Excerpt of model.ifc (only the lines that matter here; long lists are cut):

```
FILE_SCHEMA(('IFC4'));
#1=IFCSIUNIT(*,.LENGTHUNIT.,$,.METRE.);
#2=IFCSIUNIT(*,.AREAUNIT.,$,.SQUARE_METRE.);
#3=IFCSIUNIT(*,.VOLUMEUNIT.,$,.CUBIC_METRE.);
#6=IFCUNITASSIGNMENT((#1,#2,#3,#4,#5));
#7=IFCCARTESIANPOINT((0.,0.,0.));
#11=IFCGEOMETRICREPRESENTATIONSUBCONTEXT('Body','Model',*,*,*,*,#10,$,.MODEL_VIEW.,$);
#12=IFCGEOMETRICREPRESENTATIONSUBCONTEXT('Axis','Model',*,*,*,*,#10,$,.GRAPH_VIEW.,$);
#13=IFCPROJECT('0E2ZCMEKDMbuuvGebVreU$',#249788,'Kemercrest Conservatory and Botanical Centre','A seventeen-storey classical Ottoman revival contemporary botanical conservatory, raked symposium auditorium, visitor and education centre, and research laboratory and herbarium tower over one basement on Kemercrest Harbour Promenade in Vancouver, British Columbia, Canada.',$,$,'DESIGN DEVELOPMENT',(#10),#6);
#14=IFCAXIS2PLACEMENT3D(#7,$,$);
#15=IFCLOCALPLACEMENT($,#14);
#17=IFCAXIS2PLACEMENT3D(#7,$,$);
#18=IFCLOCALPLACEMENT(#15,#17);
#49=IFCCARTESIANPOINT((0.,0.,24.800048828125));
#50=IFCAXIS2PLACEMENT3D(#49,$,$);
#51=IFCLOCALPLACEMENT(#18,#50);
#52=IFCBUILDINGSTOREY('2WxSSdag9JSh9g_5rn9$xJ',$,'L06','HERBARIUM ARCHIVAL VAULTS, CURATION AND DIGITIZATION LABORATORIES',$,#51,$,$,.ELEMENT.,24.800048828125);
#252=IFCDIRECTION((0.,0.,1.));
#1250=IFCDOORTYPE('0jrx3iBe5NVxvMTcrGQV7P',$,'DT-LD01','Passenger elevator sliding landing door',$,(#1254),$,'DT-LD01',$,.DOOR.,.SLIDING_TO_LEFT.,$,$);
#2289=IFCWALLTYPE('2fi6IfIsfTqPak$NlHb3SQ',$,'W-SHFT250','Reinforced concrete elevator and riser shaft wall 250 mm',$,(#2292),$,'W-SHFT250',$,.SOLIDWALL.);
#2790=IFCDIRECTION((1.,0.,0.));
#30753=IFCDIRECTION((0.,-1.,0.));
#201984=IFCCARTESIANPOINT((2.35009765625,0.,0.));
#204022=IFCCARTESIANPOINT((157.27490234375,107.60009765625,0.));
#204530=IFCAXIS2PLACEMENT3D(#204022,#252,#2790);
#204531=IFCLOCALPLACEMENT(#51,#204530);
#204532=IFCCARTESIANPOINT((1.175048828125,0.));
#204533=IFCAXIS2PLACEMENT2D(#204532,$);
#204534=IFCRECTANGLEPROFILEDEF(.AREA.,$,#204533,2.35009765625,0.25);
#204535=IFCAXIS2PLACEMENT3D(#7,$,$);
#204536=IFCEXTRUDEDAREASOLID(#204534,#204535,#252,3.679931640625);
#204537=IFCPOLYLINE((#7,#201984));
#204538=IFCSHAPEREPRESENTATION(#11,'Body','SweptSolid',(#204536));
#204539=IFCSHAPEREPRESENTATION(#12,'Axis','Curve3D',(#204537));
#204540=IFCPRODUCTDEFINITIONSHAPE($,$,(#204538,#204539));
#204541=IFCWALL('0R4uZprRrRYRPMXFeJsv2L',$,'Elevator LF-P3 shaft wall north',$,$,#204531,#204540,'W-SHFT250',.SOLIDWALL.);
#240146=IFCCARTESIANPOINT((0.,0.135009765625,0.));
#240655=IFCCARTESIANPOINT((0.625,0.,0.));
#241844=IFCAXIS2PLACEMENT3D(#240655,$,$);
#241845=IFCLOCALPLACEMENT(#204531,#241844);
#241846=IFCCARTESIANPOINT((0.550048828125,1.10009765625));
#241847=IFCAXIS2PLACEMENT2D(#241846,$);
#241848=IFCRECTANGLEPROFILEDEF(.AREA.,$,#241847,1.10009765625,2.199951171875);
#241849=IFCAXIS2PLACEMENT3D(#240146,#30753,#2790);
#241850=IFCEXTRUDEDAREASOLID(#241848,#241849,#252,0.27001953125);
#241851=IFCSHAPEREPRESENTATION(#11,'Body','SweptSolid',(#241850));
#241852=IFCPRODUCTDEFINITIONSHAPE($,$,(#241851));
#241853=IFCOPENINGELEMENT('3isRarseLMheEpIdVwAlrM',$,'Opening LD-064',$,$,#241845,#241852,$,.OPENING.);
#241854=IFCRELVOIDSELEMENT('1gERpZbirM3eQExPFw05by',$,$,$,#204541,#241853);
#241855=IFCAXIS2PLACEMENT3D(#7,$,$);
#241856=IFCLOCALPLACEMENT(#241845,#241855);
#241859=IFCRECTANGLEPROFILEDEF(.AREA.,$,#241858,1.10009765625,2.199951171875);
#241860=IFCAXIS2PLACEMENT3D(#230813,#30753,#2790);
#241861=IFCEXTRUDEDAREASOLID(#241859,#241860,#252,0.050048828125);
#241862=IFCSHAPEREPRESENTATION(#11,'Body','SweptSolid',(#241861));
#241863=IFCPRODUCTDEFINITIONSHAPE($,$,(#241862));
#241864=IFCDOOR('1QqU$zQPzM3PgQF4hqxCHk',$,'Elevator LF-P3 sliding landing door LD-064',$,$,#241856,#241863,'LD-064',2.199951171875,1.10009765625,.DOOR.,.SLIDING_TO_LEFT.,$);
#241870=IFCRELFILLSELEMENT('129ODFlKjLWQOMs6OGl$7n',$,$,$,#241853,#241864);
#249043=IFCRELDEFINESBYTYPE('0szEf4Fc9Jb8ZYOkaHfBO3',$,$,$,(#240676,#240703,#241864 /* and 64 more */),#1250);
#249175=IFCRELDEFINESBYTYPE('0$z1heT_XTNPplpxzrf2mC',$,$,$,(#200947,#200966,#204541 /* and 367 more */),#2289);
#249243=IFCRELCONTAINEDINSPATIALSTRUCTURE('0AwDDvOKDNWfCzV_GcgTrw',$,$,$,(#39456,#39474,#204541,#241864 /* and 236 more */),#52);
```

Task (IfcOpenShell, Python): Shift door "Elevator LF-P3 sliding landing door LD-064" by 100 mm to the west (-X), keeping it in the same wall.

```python
import ifcopenshell
import ifcopenshell.api.geometry
import ifcopenshell.util.placement
import ifcopenshell.util.unit

model = ifcopenshell.open("model.ifc")
unit_scale = ifcopenshell.util.unit.calculate_unit_scale(model)

door = model.by_id(241864)
opening = door.FillsVoids[0].RelatingOpeningElement
wall = opening.VoidsElements[0].RelatingBuildingElement

wall_matrix = ifcopenshell.util.placement.get_local_placement(wall.ObjectPlacement)
shift = wall_matrix[:3, 0] * -0.1 / unit_scale
before = ifcopenshell.util.placement.get_local_placement(door.ObjectPlacement)[:3, 3].copy()

# The door is placed relative to its opening, so it follows when the opening moves.
matrix = ifcopenshell.util.placement.get_local_placement(opening.ObjectPlacement)
matrix[:3, 3] += shift
ifcopenshell.api.geometry.edit_object_placement(
    model, product=opening, matrix=matrix, is_si=False, should_transform_children=True
)

after = ifcopenshell.util.placement.get_local_placement(door.ObjectPlacement)[:3, 3]
print("door moved by", (after - before).round(3) + 0.0)

model.write("model_updated.ifc")
```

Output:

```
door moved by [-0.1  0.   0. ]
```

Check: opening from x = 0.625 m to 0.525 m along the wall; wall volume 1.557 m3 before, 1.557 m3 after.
